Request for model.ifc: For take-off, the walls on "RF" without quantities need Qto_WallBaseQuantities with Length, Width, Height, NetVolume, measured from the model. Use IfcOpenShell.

First a look at what the model holds.

```python
import ifcopenshell
import ifcopenshell.util.element
import ifcopenshell.util.unit

model = ifcopenshell.open("model.ifc")
print(model.schema)
for unit_type in ("LENGTHUNIT", "AREAUNIT", "VOLUMEUNIT"):
    print(unit_type, ifcopenshell.util.unit.calculate_unit_scale(model, unit_type))
storey = next(s for s in model.by_type("IfcBuildingStorey") if s.Name == "RF")
walls = [e for e in ifcopenshell.util.element.get_decomposition(storey) if e.is_a("IfcWall")]
for e in sorted(walls, key=lambda e: e.id()):
    print(e.id(), e.is_a(), e.Name, list(ifcopenshell.util.element.get_psets(e, qtos_only=True)), sep=" | ")
```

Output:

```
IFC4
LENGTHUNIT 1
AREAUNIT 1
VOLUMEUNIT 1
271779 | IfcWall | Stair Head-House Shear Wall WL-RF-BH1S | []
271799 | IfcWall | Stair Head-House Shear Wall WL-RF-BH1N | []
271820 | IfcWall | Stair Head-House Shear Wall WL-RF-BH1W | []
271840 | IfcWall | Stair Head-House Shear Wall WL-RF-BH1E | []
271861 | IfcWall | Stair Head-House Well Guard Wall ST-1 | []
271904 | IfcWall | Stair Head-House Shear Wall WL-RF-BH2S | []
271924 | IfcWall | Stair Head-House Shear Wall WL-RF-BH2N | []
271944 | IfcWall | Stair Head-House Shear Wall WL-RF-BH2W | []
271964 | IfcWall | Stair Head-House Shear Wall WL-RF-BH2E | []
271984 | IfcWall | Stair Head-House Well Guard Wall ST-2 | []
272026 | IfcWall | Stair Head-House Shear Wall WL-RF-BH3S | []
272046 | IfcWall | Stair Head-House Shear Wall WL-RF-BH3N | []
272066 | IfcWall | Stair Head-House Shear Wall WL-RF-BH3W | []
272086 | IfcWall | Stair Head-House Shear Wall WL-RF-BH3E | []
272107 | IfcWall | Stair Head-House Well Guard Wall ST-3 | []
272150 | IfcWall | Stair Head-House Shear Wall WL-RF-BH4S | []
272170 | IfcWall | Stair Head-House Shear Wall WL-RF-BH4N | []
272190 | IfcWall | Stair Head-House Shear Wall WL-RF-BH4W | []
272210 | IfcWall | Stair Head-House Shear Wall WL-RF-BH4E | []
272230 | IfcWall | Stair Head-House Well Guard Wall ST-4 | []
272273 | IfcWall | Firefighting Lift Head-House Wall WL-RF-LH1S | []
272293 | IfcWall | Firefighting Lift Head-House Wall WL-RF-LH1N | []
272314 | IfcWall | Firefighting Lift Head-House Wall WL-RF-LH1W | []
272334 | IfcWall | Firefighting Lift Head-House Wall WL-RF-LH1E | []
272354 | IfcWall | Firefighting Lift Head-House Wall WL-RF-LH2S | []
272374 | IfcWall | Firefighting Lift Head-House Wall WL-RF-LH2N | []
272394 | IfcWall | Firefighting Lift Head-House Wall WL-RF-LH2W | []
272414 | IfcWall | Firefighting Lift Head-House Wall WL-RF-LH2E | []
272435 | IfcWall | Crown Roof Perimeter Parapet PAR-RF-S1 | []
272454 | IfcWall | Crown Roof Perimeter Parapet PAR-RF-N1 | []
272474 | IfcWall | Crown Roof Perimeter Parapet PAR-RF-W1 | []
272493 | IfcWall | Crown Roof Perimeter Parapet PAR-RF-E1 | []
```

```python
import ifcopenshell
import ifcopenshell.api.pset
import ifcopenshell.geom
import ifcopenshell.util.element
import ifcopenshell.util.shape
import ifcopenshell.util.unit

model = ifcopenshell.open("model.ifc")
unit_scale = ifcopenshell.util.unit.calculate_unit_scale(model)
volume_scale = ifcopenshell.util.unit.calculate_unit_scale(model, "VOLUMEUNIT")
settings = ifcopenshell.geom.settings()

storey = next(s for s in model.by_type("IfcBuildingStorey") if s.Name == "RF")
walls = [e for e in ifcopenshell.util.element.get_decomposition(storey) if e.is_a("IfcWall")]

for e in sorted(walls, key=lambda e: e.id()):
    if ifcopenshell.util.element.get_psets(e, qtos_only=True, should_inherit=False):
        continue
    # Geometry comes back in metres, in the element's own axes.
    shape = ifcopenshell.geom.create_shape(settings, e)
    values = {
        "Length": ifcopenshell.util.shape.get_x(shape.geometry) / unit_scale,
        "Width": ifcopenshell.util.shape.get_y(shape.geometry) / unit_scale,
        "Height": ifcopenshell.util.shape.get_z(shape.geometry) / unit_scale,
        "NetVolume": ifcopenshell.util.shape.get_volume(shape.geometry) / volume_scale,
    }
    qto = ifcopenshell.api.pset.add_qto(model, product=e, name="Qto_WallBaseQuantities")
    ifcopenshell.api.pset.edit_qto(model, qto=qto, properties=values)
    print(e.id(), {k: round(v, 3) for k, v in values.items()})

model.write("model_rev.ifc")
```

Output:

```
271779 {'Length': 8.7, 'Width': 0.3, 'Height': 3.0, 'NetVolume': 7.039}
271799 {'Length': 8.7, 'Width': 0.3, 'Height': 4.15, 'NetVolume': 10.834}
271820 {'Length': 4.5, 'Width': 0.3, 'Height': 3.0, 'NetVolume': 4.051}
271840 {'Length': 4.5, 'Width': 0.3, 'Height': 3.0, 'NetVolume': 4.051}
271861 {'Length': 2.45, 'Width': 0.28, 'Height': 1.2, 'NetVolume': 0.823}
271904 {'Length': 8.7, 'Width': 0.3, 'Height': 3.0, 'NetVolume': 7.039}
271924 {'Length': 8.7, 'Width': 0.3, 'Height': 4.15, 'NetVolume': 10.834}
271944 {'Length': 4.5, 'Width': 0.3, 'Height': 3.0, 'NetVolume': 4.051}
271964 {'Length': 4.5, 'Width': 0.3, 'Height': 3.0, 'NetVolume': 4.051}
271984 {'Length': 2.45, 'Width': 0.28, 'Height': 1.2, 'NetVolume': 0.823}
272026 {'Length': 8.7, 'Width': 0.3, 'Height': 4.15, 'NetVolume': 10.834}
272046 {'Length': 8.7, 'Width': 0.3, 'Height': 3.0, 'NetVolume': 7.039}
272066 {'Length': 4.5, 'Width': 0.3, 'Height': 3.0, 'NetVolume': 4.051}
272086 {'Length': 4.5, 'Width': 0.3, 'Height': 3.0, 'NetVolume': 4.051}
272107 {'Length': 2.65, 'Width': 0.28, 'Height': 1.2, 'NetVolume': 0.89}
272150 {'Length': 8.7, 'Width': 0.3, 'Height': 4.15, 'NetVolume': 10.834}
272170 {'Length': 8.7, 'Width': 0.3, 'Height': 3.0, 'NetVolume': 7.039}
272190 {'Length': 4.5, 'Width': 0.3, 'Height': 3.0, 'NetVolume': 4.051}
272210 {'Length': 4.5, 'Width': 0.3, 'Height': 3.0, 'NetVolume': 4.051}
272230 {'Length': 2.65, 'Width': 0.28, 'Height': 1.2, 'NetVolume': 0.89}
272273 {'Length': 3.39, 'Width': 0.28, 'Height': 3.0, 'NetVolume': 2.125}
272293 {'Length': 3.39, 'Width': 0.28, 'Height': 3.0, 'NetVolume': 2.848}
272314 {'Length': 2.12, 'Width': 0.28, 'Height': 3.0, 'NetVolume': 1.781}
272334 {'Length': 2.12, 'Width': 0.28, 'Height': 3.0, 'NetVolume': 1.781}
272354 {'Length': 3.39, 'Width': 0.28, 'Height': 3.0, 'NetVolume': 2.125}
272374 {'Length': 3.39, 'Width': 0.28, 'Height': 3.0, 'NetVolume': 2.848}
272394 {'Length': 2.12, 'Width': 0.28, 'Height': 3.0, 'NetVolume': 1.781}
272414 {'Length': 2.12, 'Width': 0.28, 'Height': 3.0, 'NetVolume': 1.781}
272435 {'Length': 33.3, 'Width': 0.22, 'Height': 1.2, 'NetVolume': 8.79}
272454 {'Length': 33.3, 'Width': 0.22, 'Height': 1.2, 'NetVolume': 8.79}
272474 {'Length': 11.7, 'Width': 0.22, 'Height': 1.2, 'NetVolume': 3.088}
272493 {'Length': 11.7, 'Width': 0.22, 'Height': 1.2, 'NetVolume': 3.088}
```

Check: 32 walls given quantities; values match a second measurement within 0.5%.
